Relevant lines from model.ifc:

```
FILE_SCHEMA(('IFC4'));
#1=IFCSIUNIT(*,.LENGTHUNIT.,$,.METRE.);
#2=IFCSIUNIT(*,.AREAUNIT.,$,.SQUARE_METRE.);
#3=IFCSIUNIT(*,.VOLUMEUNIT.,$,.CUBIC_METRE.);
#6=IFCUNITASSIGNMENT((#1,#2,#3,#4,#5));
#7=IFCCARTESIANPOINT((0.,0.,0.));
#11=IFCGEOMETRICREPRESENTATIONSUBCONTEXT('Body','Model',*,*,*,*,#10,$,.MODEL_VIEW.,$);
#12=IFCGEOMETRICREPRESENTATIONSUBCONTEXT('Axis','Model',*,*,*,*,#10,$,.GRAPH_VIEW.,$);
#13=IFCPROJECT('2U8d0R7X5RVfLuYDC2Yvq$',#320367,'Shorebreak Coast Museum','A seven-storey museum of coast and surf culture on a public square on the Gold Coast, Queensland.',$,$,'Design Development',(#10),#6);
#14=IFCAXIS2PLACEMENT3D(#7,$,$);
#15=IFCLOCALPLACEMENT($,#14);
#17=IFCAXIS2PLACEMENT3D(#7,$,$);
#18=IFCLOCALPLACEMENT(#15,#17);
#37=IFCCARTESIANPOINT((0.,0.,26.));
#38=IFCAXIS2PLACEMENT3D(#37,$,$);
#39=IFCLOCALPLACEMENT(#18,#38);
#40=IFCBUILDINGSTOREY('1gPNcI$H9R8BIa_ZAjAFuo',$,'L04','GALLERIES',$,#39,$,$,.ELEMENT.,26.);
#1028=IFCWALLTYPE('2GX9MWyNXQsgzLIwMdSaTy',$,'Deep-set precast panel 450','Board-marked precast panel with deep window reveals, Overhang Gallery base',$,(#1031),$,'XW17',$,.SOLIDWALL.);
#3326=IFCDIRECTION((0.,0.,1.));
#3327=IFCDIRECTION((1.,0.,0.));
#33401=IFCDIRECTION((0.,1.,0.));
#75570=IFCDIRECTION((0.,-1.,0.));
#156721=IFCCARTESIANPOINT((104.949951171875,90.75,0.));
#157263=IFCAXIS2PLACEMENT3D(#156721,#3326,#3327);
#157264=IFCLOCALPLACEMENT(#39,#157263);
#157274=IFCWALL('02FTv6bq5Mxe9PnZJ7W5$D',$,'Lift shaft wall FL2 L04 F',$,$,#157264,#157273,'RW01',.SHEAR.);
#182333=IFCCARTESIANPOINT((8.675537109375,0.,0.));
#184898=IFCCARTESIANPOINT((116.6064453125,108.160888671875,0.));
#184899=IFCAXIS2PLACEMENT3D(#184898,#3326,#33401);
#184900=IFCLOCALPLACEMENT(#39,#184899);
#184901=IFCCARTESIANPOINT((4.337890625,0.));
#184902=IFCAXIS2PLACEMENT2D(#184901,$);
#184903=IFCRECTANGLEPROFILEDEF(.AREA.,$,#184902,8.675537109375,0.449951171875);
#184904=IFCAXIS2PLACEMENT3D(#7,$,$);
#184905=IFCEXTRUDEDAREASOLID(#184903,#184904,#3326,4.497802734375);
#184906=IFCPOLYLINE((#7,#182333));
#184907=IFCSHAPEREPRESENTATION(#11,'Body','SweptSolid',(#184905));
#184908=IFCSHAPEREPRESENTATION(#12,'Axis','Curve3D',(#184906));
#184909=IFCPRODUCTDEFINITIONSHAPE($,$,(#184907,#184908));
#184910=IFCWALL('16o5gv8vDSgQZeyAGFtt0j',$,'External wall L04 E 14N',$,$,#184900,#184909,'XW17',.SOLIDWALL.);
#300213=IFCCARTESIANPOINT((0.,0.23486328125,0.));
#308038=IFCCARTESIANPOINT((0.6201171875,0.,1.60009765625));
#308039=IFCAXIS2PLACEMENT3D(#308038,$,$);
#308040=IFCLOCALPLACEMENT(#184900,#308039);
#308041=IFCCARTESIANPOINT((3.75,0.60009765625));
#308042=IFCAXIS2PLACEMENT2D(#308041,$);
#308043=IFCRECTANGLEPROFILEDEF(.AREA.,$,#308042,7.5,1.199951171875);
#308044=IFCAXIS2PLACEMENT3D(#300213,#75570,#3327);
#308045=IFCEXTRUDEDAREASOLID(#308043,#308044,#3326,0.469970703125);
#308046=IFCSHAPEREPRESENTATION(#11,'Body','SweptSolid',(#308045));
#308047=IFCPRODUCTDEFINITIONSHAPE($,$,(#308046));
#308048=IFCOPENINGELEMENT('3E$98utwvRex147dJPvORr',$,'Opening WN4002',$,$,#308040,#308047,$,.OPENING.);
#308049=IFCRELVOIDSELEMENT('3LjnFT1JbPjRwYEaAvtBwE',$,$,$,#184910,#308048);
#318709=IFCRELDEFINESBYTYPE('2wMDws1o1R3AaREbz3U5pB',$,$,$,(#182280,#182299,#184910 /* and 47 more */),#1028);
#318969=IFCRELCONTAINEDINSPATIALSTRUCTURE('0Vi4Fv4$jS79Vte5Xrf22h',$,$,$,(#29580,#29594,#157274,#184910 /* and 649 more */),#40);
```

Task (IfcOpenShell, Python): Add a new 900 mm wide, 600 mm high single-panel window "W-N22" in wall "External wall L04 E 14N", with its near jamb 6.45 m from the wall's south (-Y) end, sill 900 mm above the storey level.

```python
import numpy as np
import ifcopenshell
import ifcopenshell.api.feature
import ifcopenshell.api.geometry
import ifcopenshell.api.root
import ifcopenshell.api.spatial
import ifcopenshell.geom
import ifcopenshell.util.element
import ifcopenshell.util.placement
import ifcopenshell.util.representation
import ifcopenshell.util.shape
import ifcopenshell.util.unit

model = ifcopenshell.open("model.ifc")
unit_scale = ifcopenshell.util.unit.calculate_unit_scale(model)
settings = ifcopenshell.geom.settings()


def volume(element):
    """Net volume in cubic metres, openings subtracted."""
    shape = ifcopenshell.geom.create_shape(settings, element)
    return ifcopenshell.util.shape.get_volume(shape.geometry)


wall = model.by_id(184910)
storey = ifcopenshell.util.element.get_container(wall, ifc_class="IfcBuildingStorey")
context = ifcopenshell.util.representation.get_context(model, "Model", "Body", "MODEL_VIEW")
before = volume(wall)

width, height, from_end, sill = 0.9, 0.6, 6.45, 0.9  # metres

# The wall runs along its own X axis, and the end named is its -X end.
wall_shape = ifcopenshell.geom.create_shape(settings, wall)
x, y, z = ifcopenshell.util.shape.get_vertices(wall_shape.geometry).T
start = x.min() + from_end
face, thickness = float(y.min()), float(y.max() - y.min())
wall_matrix = ifcopenshell.util.placement.get_local_placement(wall.ObjectPlacement)
level = ifcopenshell.util.placement.get_local_placement(storey.ObjectPlacement)[2, 3]


def in_wall(x, y):
    """Placement at x, y metres in the wall's axes, at sill height."""
    matrix = wall_matrix.copy()
    matrix[:, 3] = wall_matrix @ np.array([x / unit_scale, y / unit_scale, 0.0, 1.0])
    matrix[2, 3] = level + sill / unit_scale
    return matrix


# Opening: a box that overshoots both wall faces by 50 mm.
opening = ifcopenshell.api.root.create_entity(model, ifc_class="IfcOpeningElement", predefined_type="OPENING")
box = ifcopenshell.api.geometry.add_wall_representation(
    model, context=context, length=width, height=height, thickness=thickness + 0.1
)
ifcopenshell.api.geometry.assign_representation(model, product=opening, representation=box)
ifcopenshell.api.geometry.edit_object_placement(model, product=opening, matrix=in_wall(start, face - 0.05), is_si=False)
ifcopenshell.api.feature.add_feature(model, feature=opening, element=wall)

window = ifcopenshell.api.root.create_entity(model, ifc_class="IfcWindow", name="W-N22", predefined_type="WINDOW")
window.OverallWidth, window.OverallHeight = width / unit_scale, height / unit_scale
window.PartitioningType = "SINGLE_PANEL"
body = ifcopenshell.api.geometry.add_window_representation(
    model,
    context=context,
    overall_width=window.OverallWidth,
    overall_height=window.OverallHeight,
    partition_type="SINGLE_PANEL",
)
ifcopenshell.api.geometry.assign_representation(model, product=window, representation=body)
ifcopenshell.api.spatial.assign_container(model, products=[window], relating_structure=storey)
ifcopenshell.api.feature.add_filling(model, opening=opening, element=window)

# Centre the window in the wall's thickness.
ifcopenshell.api.geometry.edit_object_placement(model, product=window, matrix=in_wall(start, face), is_si=False)
window_shape = ifcopenshell.geom.create_shape(settings, window)
depth = ifcopenshell.util.shape.get_vertices(window_shape.geometry)[:, 1]
offset = face + thickness / 2 - (depth.min() + depth.max()) / 2
ifcopenshell.api.geometry.edit_object_placement(model, product=window, matrix=in_wall(start, offset), is_si=False)

after = volume(wall)

print(f"wall volume {before:.3f} -> {after:.3f} m3")

model.write("model_edited.ifc")
```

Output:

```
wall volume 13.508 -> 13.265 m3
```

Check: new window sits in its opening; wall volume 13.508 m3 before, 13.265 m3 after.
